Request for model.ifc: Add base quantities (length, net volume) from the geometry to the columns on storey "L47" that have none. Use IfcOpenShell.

First a look at what the model holds.

```python
import ifcopenshell
import ifcopenshell.util.element
import ifcopenshell.util.unit

model = ifcopenshell.open("model.ifc")
print(model.schema)
for unit_type in ("LENGTHUNIT", "AREAUNIT", "VOLUMEUNIT"):
    print(unit_type, ifcopenshell.util.unit.calculate_unit_scale(model, unit_type))
storey = next(s for s in model.by_type("IfcBuildingStorey") if s.Name == "L47")
columns = [e for e in ifcopenshell.util.element.get_decomposition(storey) if e.is_a("IfcColumn")]
for e in sorted(columns, key=lambda e: e.id()):
    print(e.id(), e.is_a(), e.Name, list(ifcopenshell.util.element.get_psets(e, qtos_only=True)), sep=" | ")
```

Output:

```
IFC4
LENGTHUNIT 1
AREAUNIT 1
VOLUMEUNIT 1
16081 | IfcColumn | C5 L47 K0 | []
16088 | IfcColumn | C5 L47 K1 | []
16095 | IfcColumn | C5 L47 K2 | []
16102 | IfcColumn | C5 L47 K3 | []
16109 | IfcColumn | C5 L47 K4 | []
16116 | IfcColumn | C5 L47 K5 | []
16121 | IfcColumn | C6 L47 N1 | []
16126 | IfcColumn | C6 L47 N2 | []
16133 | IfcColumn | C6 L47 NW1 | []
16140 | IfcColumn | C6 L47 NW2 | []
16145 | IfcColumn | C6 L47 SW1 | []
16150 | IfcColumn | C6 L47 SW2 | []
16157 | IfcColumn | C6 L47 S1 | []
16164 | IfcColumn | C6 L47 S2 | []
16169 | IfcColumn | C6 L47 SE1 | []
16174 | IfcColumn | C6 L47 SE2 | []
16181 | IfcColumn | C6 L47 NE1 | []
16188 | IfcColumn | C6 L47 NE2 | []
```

```python
import ifcopenshell
import ifcopenshell.api.pset
import ifcopenshell.geom
import ifcopenshell.util.element
import ifcopenshell.util.shape
import ifcopenshell.util.unit

model = ifcopenshell.open("model.ifc")
unit_scale = ifcopenshell.util.unit.calculate_unit_scale(model)
volume_scale = ifcopenshell.util.unit.calculate_unit_scale(model, "VOLUMEUNIT")
settings = ifcopenshell.geom.settings()

storey = next(s for s in model.by_type("IfcBuildingStorey") if s.Name == "L47")
columns = [e for e in ifcopenshell.util.element.get_decomposition(storey) if e.is_a("IfcColumn")]

for e in sorted(columns, key=lambda e: e.id()):
    if ifcopenshell.util.element.get_psets(e, qtos_only=True, should_inherit=False):
        continue
    # Geometry comes back in metres, in the element's own axes.
    shape = ifcopenshell.geom.create_shape(settings, e)
    values = {
        "Length": ifcopenshell.util.shape.get_z(shape.geometry) / unit_scale,
        "NetVolume": ifcopenshell.util.shape.get_volume(shape.geometry) / volume_scale,
    }
    qto = ifcopenshell.api.pset.add_qto(model, product=e, name="Qto_ColumnBaseQuantities")
    ifcopenshell.api.pset.edit_qto(model, qto=qto, properties=values)
    print(e.id(), {k: round(v, 3) for k, v in values.items()})

model.write("model_edited.ifc")
```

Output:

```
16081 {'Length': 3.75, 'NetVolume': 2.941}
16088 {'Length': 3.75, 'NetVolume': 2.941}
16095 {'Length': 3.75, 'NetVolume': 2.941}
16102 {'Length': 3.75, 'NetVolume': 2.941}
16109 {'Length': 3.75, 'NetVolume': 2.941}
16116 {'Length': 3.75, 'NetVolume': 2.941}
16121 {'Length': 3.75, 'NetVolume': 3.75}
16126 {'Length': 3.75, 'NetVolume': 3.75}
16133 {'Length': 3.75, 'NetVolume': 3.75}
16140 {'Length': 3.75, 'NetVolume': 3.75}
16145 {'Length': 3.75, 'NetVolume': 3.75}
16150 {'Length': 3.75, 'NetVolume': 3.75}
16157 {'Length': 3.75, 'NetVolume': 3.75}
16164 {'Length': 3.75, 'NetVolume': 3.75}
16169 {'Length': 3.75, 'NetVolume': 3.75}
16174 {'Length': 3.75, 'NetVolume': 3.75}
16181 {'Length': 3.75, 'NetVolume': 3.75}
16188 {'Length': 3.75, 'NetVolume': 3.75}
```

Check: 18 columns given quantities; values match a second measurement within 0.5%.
